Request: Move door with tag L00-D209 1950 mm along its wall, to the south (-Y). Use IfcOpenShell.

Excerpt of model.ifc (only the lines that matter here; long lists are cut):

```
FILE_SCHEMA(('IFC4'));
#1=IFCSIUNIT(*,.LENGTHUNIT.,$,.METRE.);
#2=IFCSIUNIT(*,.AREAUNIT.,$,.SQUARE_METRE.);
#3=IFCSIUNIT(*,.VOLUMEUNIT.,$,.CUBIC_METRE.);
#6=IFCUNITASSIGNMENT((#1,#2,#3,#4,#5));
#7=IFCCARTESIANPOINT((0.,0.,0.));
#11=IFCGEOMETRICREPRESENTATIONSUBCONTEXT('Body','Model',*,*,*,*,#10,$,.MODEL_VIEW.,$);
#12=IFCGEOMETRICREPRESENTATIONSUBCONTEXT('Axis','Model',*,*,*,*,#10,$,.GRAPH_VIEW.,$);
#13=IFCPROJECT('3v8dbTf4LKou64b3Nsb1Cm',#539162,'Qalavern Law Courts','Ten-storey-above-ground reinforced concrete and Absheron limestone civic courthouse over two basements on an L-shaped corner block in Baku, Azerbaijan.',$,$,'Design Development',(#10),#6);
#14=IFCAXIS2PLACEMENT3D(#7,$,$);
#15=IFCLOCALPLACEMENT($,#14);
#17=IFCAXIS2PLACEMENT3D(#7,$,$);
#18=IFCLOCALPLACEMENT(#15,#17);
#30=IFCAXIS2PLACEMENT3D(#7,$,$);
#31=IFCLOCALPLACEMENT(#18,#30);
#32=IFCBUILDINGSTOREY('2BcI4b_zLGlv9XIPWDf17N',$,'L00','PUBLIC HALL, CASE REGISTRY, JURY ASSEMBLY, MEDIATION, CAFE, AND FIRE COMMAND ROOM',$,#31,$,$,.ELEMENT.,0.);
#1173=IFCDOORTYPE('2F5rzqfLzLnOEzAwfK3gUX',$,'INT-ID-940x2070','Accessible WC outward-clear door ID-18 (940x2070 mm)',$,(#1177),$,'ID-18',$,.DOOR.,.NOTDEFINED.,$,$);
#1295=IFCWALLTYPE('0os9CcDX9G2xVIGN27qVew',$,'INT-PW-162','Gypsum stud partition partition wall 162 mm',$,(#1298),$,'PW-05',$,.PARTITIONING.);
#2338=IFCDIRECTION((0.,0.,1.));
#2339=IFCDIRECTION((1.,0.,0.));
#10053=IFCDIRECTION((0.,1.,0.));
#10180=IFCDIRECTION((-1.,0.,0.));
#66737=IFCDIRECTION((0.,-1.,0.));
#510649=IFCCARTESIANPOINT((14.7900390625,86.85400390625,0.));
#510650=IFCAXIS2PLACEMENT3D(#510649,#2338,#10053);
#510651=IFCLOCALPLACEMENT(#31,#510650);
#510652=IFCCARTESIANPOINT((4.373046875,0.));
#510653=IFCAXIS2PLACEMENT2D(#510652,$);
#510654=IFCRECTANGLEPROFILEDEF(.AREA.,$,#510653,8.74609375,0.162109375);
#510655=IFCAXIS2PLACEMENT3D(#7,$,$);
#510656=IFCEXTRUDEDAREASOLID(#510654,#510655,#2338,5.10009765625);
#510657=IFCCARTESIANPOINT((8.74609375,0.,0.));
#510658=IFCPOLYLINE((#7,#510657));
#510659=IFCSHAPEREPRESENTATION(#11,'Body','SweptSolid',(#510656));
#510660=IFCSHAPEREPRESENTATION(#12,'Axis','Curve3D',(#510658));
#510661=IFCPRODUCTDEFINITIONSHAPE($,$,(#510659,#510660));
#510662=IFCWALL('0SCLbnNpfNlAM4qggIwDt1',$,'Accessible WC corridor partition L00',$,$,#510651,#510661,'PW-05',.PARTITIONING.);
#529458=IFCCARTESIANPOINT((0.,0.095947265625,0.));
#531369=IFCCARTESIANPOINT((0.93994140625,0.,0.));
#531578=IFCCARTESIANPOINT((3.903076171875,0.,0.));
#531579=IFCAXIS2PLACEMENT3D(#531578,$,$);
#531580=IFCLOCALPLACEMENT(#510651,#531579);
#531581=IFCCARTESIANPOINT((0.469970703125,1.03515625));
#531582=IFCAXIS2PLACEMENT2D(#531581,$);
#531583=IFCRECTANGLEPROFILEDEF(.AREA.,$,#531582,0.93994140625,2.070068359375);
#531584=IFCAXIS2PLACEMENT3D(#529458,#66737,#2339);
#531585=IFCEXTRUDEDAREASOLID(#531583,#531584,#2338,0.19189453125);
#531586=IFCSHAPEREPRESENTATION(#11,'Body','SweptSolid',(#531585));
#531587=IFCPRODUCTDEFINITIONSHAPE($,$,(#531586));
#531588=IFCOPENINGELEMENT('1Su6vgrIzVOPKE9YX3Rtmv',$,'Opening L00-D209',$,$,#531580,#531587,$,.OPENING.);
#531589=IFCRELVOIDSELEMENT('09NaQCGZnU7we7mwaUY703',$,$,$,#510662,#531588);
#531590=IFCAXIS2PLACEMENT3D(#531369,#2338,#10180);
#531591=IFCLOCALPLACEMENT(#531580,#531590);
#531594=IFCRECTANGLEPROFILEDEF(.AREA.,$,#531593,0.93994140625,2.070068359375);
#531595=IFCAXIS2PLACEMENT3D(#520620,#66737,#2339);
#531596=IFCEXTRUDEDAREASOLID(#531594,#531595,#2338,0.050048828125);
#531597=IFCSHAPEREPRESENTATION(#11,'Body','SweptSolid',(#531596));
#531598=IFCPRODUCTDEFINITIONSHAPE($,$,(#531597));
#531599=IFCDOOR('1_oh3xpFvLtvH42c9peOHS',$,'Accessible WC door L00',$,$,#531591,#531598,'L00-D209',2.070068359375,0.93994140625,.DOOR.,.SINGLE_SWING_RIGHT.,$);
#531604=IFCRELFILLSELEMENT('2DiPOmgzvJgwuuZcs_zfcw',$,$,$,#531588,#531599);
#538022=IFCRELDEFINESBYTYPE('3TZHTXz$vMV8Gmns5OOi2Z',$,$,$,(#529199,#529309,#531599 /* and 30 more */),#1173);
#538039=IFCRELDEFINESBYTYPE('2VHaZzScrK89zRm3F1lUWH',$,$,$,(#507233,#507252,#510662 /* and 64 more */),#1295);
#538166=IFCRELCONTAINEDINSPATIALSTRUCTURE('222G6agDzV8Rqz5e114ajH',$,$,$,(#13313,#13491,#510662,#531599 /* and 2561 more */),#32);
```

```python
import ifcopenshell
import ifcopenshell.api.geometry
import ifcopenshell.util.placement
import ifcopenshell.util.unit

model = ifcopenshell.open("model.ifc")
unit_scale = ifcopenshell.util.unit.calculate_unit_scale(model)

door = model.by_guid("1_oh3xpFvLtvH42c9peOHS")
opening = door.FillsVoids[0].RelatingOpeningElement
wall = opening.VoidsElements[0].RelatingBuildingElement

wall_matrix = ifcopenshell.util.placement.get_local_placement(wall.ObjectPlacement)
shift = wall_matrix[:3, 0] * -1.95 / unit_scale
before = ifcopenshell.util.placement.get_local_placement(door.ObjectPlacement)[:3, 3].copy()

# The door is placed relative to its opening, so it follows when the opening moves.
matrix = ifcopenshell.util.placement.get_local_placement(opening.ObjectPlacement)
matrix[:3, 3] += shift
ifcopenshell.api.geometry.edit_object_placement(
    model, product=opening, matrix=matrix, is_si=False, should_transform_children=True
)

after = ifcopenshell.util.placement.get_local_placement(door.ObjectPlacement)[:3, 3]
print("door moved by", (after - before).round(3) + 0.0)

model.write("model_updated.ifc")
```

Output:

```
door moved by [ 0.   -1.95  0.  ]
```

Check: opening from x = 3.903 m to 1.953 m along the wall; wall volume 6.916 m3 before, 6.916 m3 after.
